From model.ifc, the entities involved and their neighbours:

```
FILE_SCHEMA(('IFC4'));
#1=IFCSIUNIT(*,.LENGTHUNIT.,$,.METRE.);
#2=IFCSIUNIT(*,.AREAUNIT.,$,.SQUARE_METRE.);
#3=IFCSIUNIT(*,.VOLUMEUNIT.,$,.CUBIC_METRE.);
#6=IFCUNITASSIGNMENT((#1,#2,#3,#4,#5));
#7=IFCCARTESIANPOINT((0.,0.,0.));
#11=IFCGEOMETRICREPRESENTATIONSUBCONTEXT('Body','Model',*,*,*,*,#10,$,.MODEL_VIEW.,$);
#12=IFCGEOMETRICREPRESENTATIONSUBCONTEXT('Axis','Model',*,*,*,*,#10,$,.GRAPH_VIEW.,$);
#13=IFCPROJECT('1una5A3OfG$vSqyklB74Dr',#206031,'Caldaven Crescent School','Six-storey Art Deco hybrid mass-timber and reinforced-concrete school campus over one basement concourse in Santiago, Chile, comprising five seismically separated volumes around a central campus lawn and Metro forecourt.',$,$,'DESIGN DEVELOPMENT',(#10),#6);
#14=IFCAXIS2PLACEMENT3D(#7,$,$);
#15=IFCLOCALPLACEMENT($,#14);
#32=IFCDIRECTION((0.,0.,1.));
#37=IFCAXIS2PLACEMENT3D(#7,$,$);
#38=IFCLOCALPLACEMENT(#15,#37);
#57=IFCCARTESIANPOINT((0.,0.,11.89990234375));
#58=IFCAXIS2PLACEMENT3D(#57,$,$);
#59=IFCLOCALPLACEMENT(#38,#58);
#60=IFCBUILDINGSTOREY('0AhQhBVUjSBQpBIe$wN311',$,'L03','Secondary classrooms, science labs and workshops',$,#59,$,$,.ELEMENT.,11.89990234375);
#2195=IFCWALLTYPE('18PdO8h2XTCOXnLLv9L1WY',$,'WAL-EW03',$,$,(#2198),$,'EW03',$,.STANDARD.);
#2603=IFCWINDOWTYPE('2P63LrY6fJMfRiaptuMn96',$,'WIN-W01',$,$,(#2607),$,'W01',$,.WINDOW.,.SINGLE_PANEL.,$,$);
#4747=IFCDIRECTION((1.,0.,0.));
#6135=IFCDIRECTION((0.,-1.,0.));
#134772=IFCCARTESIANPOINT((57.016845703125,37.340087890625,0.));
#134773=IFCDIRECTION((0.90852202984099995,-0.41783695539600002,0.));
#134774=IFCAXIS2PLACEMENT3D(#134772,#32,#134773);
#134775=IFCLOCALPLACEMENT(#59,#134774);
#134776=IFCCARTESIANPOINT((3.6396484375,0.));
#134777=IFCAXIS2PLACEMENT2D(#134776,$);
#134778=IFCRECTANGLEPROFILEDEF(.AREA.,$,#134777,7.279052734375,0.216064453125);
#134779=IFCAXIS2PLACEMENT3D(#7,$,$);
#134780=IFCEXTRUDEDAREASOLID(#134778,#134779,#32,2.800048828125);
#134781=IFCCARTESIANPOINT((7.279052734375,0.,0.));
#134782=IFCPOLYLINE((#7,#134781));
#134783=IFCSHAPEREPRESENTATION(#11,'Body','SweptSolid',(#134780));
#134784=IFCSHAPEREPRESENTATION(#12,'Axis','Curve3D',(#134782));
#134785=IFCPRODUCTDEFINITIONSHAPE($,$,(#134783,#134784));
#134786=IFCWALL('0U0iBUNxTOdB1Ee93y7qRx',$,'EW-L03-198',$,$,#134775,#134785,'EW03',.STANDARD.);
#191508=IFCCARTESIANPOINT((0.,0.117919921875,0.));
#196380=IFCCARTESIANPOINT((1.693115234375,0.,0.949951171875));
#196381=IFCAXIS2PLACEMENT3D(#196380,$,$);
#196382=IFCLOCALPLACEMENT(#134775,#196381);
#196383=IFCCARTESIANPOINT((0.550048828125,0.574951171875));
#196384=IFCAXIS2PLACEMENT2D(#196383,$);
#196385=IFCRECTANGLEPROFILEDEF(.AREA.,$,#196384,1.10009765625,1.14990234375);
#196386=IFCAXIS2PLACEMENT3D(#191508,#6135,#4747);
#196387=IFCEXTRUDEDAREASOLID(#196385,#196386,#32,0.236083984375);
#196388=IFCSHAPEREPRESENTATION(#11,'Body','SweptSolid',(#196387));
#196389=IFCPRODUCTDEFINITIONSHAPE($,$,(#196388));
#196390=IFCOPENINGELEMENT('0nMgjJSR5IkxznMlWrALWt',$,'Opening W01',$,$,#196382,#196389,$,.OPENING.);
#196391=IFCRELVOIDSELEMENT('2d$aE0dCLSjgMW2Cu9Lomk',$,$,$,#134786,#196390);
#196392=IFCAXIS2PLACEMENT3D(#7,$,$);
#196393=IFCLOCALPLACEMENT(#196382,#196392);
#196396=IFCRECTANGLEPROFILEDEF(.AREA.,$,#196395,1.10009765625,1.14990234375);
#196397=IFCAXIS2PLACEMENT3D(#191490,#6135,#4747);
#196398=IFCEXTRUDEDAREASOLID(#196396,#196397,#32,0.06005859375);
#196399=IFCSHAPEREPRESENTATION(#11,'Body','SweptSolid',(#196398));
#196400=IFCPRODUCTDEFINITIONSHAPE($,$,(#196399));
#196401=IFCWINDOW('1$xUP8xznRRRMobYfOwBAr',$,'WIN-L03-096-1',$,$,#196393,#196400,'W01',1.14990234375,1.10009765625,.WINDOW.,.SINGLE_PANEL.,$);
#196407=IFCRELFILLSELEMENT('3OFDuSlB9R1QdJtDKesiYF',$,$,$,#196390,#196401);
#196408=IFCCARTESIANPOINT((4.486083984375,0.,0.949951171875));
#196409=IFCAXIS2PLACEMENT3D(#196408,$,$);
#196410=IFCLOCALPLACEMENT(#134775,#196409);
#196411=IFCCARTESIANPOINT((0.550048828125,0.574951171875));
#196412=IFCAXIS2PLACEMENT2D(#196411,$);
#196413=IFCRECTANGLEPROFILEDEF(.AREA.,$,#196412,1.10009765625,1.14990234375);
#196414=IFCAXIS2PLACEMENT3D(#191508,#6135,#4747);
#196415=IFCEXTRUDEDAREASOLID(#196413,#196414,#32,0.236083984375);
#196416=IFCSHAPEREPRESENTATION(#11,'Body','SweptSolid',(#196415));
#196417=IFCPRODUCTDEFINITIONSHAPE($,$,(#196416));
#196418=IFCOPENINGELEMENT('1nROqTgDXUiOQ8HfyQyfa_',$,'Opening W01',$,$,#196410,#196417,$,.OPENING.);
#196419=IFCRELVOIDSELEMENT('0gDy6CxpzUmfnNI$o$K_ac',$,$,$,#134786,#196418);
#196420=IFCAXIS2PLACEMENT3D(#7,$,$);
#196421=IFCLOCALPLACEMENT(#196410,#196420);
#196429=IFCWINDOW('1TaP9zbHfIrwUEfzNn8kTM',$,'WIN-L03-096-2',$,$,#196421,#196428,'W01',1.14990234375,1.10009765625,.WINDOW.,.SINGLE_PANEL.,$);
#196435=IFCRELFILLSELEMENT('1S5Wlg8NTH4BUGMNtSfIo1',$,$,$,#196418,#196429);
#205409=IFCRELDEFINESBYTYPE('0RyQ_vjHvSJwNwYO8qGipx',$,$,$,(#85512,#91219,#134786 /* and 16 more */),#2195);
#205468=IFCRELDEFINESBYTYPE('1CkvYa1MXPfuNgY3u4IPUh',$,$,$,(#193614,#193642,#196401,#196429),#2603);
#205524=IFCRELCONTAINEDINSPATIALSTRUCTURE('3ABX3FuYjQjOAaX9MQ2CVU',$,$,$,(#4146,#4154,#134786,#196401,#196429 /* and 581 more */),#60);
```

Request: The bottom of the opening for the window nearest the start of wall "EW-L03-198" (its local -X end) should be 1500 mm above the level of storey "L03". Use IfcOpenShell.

```python
import numpy as np
import ifcopenshell
import ifcopenshell.api.geometry
import ifcopenshell.geom
import ifcopenshell.util.element
import ifcopenshell.util.placement
import ifcopenshell.util.shape
import ifcopenshell.util.unit

model = ifcopenshell.open("model.ifc")
unit_scale = ifcopenshell.util.unit.calculate_unit_scale(model)

window = model.by_id(196401)
opening = window.FillsVoids[0].RelatingOpeningElement
storey = ifcopenshell.util.element.get_container(window, ifc_class="IfcBuildingStorey")
level = ifcopenshell.util.placement.get_local_placement(storey.ObjectPlacement)[2, 3]

# The opening's origin need not be at the sill, so measure its lowest point.
shape = ifcopenshell.geom.create_shape(ifcopenshell.geom.settings(), opening)
bottom = ifcopenshell.util.shape.get_shape_bottom_elevation(shape, shape.geometry) / unit_scale
dz = level + 1.5 - bottom

shift = np.array([0.0, 0.0, dz])
# The window is placed relative to its opening, so it follows when the opening moves.
matrix = ifcopenshell.util.placement.get_local_placement(opening.ObjectPlacement)
matrix[:3, 3] += shift
ifcopenshell.api.geometry.edit_object_placement(
    model, product=opening, matrix=matrix, is_si=False, should_transform_children=True
)

print(f"moved by {dz * unit_scale:+.3f} m")

model.write("model_edited.ifc")
```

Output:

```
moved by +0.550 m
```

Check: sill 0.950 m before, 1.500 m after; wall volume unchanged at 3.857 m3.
